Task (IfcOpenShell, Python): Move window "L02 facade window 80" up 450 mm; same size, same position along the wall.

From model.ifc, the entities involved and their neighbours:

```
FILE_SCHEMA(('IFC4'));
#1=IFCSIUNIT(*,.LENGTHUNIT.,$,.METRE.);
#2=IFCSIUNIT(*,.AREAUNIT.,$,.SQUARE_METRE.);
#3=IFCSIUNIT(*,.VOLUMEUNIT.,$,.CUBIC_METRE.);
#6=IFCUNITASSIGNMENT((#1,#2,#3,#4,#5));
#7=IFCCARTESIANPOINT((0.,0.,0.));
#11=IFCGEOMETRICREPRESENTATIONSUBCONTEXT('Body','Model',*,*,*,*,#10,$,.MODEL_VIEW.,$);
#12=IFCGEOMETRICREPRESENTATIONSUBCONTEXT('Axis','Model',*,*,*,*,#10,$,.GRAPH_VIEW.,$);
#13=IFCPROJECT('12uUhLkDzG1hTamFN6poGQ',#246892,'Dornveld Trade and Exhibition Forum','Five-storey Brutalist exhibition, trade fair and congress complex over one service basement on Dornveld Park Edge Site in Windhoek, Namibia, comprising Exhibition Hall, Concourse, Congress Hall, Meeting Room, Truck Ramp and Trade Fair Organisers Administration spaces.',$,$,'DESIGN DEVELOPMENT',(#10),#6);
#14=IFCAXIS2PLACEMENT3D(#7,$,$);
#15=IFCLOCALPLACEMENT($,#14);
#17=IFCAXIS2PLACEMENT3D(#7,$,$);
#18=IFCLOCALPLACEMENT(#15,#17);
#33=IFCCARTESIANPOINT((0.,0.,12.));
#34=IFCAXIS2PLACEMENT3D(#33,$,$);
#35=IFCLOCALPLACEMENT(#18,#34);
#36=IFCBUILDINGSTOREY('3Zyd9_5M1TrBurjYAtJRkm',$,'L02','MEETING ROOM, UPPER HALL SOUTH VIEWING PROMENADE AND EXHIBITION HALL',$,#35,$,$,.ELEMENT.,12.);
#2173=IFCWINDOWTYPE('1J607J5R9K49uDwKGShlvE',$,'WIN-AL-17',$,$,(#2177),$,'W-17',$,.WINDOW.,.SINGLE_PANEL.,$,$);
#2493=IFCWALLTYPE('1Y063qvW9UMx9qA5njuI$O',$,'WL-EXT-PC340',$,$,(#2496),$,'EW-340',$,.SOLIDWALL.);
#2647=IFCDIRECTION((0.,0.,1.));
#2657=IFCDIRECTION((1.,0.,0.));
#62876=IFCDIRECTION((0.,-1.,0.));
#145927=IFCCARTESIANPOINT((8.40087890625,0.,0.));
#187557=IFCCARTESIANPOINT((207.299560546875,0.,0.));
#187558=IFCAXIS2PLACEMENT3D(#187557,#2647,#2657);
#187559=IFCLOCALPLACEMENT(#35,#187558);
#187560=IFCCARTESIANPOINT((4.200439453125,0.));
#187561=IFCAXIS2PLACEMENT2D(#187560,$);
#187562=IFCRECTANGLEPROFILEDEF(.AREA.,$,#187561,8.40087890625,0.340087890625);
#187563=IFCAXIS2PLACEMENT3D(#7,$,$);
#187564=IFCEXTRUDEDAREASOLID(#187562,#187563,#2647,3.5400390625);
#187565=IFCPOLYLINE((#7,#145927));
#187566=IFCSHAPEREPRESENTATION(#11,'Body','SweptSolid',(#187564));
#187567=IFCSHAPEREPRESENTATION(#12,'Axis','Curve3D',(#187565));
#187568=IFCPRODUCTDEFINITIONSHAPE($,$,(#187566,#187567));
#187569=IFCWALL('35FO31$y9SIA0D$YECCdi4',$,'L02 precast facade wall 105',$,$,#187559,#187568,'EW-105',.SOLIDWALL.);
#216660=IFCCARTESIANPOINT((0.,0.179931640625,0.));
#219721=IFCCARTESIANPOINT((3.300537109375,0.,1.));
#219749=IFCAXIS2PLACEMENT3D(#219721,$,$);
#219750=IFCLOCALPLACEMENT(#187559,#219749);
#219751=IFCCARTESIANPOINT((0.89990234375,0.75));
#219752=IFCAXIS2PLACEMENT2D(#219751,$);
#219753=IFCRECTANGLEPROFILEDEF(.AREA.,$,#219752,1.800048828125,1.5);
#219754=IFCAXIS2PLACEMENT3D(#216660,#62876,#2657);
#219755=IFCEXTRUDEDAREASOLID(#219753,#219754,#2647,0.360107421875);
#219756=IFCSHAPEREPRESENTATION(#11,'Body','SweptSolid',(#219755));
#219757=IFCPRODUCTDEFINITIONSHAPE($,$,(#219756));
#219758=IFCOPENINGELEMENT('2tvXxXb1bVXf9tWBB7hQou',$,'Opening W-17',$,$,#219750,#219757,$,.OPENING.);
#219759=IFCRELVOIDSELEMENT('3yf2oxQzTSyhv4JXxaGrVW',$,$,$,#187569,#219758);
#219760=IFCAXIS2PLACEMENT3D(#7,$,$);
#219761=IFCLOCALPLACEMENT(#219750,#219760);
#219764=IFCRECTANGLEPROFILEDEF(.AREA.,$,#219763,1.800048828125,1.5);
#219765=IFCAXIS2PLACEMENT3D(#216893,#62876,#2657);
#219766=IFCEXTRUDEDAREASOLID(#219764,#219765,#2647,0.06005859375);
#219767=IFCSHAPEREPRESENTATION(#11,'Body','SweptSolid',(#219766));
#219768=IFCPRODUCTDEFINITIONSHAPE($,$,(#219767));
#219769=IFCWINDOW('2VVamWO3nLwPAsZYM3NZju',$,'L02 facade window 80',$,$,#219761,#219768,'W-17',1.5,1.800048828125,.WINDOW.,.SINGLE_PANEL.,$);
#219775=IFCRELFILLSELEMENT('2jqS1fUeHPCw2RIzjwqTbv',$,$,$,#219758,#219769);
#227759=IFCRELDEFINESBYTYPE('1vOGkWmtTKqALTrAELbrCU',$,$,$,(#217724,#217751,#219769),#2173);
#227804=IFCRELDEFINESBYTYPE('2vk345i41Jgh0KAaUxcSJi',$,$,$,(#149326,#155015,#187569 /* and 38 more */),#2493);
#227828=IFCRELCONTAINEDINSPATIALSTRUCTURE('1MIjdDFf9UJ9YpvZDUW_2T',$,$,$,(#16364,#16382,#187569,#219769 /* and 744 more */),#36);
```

```python
import numpy as np
import ifcopenshell
import ifcopenshell.api.geometry
import ifcopenshell.util.placement
import ifcopenshell.util.unit

model = ifcopenshell.open("model.ifc")
unit_scale = ifcopenshell.util.unit.calculate_unit_scale(model)

window = model.by_guid("2VVamWO3nLwPAsZYM3NZju")
opening = window.FillsVoids[0].RelatingOpeningElement
dz = 0.45 / unit_scale

shift = np.array([0.0, 0.0, dz])
# The window is placed relative to its opening, so it follows when the opening moves.
matrix = ifcopenshell.util.placement.get_local_placement(opening.ObjectPlacement)
matrix[:3, 3] += shift
ifcopenshell.api.geometry.edit_object_placement(
    model, product=opening, matrix=matrix, is_si=False, should_transform_children=True
)

print(f"moved by {dz * unit_scale:+.3f} m")

model.write("model_v2.ifc")
```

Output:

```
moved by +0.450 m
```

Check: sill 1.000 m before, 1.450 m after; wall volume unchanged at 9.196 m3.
